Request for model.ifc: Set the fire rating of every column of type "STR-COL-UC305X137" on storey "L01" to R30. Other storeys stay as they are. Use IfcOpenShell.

First a look at what the model holds.

```python
import ifcopenshell
import ifcopenshell.util.element

model = ifcopenshell.open("model.ifc")
print(model.schema)
storey = next(s for s in model.by_type("IfcBuildingStorey") if s.Name == "L01")
columns = [e for e in ifcopenshell.util.element.get_decomposition(storey) if e.is_a("IfcColumn")]
seen = {}
for e in columns:
    element_type = ifcopenshell.util.element.get_type(e)
    key = (element_type.Name if element_type != e and element_type else None, ifcopenshell.util.element.get_pset(e, "Pset_ColumnCommon", "FireRating"))
    seen[key] = seen.get(key, 0) + 1
for (name, value), count in sorted(seen.items(), key=str):
    print(count, "x", name, "|", value)
```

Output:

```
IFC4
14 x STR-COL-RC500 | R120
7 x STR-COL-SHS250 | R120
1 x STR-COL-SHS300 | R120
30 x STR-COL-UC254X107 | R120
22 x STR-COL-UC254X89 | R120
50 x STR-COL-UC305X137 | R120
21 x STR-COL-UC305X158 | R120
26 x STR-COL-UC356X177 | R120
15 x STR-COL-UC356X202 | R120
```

```python
import ifcopenshell
import ifcopenshell.api.pset
import ifcopenshell.util.element

model = ifcopenshell.open("model.ifc")

storey = next(s for s in model.by_type("IfcBuildingStorey") if s.Name == "L01")
columns = [e for e in ifcopenshell.util.element.get_decomposition(storey) if e.is_a("IfcColumn")]

count = 0
for e in columns:
    element_type = ifcopenshell.util.element.get_type(e)
    if element_type in (None, e) or element_type.Name != "STR-COL-UC305X137":
        continue
    # add_pset returns the element's existing set when there is one.
    pset = ifcopenshell.api.pset.add_pset(model, product=e, name="Pset_ColumnCommon")
    ifcopenshell.api.pset.edit_pset(model, pset=pset, properties={"FireRating": "R30"})
    count += 1

print(count, "columns updated")

model.write("model-out.ifc")
```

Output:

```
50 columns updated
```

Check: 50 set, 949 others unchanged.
